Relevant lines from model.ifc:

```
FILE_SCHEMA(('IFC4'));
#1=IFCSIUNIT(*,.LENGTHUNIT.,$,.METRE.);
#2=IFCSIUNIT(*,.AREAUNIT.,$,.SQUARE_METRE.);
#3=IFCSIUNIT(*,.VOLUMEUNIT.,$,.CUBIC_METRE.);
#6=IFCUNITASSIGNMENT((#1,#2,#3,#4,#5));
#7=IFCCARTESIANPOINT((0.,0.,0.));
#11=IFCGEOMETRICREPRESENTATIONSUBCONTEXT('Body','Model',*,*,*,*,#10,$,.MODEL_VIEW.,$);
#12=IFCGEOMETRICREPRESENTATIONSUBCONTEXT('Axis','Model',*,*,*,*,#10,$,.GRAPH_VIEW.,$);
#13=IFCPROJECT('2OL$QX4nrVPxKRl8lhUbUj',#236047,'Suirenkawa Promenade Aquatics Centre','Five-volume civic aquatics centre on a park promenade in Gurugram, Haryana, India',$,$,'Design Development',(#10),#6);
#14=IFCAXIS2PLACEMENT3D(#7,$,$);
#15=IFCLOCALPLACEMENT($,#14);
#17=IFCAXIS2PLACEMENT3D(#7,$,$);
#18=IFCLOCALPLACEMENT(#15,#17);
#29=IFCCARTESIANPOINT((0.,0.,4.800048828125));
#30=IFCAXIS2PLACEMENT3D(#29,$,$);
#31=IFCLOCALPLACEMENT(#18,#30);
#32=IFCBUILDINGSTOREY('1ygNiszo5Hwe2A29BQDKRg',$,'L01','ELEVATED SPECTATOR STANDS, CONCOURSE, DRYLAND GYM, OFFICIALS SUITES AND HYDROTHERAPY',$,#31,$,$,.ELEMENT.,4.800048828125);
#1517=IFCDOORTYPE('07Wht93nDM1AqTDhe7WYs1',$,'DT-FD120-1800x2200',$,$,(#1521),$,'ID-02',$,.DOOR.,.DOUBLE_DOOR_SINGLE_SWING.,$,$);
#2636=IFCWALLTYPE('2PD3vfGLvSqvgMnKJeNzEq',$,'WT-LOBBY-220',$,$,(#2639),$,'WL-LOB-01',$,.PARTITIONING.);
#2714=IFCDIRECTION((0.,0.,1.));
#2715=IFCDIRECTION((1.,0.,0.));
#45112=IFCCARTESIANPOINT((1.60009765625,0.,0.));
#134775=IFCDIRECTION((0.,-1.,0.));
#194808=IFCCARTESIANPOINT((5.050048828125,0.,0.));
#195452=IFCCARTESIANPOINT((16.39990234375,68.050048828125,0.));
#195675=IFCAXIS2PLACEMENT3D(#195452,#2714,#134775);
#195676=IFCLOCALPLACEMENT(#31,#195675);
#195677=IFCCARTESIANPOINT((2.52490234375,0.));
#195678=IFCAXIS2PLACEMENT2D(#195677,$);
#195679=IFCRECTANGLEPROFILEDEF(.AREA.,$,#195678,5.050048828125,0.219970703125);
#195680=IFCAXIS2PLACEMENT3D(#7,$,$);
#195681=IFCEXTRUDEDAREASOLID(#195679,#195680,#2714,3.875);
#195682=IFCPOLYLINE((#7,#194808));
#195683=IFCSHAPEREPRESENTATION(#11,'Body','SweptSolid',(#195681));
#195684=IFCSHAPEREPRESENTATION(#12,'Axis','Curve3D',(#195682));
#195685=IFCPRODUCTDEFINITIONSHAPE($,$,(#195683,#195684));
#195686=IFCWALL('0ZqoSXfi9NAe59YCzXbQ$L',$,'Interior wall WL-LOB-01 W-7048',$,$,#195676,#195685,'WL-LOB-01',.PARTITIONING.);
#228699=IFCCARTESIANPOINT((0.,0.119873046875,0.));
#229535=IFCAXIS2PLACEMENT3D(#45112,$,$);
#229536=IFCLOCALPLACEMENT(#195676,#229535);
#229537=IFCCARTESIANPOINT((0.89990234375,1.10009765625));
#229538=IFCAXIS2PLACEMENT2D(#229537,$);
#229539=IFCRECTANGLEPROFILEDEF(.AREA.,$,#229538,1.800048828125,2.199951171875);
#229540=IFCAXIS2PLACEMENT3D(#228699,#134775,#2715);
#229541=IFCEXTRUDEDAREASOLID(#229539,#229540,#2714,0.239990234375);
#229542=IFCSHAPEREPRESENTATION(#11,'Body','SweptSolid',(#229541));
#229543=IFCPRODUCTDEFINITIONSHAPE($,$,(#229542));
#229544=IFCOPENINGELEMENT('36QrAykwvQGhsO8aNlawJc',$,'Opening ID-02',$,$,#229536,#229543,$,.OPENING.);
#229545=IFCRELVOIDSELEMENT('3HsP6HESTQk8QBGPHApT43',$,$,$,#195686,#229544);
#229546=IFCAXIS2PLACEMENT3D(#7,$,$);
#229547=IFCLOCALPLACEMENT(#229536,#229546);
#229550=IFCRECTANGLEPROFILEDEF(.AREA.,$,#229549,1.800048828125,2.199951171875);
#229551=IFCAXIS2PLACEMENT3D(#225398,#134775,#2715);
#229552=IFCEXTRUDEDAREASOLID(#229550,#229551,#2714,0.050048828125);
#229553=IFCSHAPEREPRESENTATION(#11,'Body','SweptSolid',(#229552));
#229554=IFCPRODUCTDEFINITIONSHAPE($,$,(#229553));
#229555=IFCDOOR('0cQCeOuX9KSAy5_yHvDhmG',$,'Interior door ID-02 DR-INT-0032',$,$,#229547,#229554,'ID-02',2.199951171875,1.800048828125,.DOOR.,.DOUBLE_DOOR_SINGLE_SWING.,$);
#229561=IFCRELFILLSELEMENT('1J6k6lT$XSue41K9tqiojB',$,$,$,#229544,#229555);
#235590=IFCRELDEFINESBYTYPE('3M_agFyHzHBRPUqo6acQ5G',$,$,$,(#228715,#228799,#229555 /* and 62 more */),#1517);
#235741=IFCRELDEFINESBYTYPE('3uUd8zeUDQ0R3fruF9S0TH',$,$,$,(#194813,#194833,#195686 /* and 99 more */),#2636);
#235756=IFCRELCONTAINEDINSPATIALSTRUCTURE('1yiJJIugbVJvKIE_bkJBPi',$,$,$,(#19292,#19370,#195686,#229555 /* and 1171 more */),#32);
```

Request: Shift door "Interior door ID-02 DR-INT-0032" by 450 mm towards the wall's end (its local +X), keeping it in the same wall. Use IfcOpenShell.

```python
import ifcopenshell
import ifcopenshell.api.geometry
import ifcopenshell.util.placement
import ifcopenshell.util.unit

model = ifcopenshell.open("model.ifc")
unit_scale = ifcopenshell.util.unit.calculate_unit_scale(model)

door = model.by_guid("0cQCeOuX9KSAy5_yHvDhmG")
opening = door.FillsVoids[0].RelatingOpeningElement
wall = opening.VoidsElements[0].RelatingBuildingElement

wall_matrix = ifcopenshell.util.placement.get_local_placement(wall.ObjectPlacement)
shift = wall_matrix[:3, 0] * 0.45 / unit_scale
before = ifcopenshell.util.placement.get_local_placement(door.ObjectPlacement)[:3, 3].copy()

# The door is placed relative to its opening, so it follows when the opening moves.
matrix = ifcopenshell.util.placement.get_local_placement(opening.ObjectPlacement)
matrix[:3, 3] += shift
ifcopenshell.api.geometry.edit_object_placement(
    model, product=opening, matrix=matrix, is_si=False, should_transform_children=True
)

after = ifcopenshell.util.placement.get_local_placement(door.ObjectPlacement)[:3, 3]
print("door moved by", (after - before).round(3) + 0.0)

model.write("model_rev.ifc")
```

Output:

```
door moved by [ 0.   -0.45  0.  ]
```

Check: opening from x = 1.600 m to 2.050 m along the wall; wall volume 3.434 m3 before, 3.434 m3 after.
